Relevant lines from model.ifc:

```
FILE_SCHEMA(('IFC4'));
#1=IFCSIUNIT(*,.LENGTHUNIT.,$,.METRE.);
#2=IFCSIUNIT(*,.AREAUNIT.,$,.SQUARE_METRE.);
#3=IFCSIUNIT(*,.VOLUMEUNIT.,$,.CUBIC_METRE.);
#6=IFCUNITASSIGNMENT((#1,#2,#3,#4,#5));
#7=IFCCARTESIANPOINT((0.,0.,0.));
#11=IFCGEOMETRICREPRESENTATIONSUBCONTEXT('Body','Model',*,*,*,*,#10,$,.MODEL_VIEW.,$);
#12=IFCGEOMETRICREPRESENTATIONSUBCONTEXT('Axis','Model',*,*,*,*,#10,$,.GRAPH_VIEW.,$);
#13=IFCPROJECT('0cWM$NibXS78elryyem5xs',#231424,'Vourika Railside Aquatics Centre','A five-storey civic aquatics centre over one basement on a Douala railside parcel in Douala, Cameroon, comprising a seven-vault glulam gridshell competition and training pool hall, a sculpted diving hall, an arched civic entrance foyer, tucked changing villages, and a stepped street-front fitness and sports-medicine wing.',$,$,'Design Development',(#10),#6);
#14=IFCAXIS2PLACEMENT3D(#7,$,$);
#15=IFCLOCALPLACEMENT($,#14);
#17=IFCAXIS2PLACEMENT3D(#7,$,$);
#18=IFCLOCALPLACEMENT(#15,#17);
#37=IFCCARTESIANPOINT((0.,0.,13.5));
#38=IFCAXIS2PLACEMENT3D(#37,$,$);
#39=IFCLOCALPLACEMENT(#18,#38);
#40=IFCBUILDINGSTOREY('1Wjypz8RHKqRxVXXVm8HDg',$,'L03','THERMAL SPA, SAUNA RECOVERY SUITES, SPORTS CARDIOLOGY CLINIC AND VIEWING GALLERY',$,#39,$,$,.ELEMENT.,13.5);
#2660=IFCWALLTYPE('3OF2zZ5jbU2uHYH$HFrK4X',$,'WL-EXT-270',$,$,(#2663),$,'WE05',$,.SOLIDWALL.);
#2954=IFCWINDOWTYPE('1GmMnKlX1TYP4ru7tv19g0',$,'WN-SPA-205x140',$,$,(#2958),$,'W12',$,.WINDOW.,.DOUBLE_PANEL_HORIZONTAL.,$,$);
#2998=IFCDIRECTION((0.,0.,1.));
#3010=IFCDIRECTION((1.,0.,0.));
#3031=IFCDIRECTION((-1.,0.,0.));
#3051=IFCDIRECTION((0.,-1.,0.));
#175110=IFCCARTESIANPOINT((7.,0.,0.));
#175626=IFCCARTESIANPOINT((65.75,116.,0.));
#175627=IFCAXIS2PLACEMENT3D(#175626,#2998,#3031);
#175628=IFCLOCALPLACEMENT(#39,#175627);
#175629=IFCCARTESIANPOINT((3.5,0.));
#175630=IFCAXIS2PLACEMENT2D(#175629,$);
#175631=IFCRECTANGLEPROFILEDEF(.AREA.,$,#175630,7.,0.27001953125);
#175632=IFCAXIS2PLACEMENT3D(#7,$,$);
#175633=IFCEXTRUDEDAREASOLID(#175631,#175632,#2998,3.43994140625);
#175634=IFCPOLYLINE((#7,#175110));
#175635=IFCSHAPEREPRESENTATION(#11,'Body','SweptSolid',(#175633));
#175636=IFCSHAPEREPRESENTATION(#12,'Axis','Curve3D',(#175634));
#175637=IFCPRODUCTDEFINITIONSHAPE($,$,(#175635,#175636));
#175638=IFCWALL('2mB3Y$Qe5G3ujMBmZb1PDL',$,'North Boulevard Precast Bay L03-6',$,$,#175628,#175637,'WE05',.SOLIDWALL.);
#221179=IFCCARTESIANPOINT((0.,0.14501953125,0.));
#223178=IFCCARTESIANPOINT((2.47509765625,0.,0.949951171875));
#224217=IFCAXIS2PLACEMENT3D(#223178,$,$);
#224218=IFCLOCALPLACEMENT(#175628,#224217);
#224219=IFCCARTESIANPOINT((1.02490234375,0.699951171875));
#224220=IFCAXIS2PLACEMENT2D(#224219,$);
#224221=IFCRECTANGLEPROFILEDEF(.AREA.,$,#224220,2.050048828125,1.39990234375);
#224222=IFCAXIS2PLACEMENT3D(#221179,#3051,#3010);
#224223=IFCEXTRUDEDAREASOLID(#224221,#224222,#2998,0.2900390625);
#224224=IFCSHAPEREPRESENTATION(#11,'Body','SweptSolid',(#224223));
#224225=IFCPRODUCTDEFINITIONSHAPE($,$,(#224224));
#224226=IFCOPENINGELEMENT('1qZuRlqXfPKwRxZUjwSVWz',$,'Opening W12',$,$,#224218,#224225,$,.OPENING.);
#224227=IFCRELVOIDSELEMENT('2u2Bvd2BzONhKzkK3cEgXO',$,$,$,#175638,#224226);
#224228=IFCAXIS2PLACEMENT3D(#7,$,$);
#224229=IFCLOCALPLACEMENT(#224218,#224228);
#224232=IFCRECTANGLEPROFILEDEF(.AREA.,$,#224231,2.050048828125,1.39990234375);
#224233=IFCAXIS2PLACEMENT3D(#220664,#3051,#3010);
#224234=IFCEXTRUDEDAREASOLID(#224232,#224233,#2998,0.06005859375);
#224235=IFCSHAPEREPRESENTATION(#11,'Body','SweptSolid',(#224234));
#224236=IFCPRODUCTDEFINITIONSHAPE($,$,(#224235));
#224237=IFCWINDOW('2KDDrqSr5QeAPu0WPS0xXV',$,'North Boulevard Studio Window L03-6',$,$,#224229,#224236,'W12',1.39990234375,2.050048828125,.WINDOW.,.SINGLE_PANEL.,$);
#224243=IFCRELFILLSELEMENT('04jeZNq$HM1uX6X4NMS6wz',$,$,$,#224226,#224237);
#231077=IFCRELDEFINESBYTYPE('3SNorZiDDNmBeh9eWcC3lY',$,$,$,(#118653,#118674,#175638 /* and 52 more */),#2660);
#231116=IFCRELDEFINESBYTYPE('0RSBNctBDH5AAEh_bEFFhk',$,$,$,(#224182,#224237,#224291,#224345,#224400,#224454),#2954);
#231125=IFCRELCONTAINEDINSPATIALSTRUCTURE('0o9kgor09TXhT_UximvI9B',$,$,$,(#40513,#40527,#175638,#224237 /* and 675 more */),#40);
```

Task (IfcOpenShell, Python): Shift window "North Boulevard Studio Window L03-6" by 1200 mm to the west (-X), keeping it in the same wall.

```python
import ifcopenshell
import ifcopenshell.api.geometry
import ifcopenshell.util.placement

model = ifcopenshell.open("model.ifc")

window = model.by_id(224237)
opening = window.FillsVoids[0].RelatingOpeningElement
wall = opening.VoidsElements[0].RelatingBuildingElement

wall_matrix = ifcopenshell.util.placement.get_local_placement(wall.ObjectPlacement)
shift = wall_matrix[:3, 0] * 1.2
before = ifcopenshell.util.placement.get_local_placement(window.ObjectPlacement)[:3, 3].copy()

# The window is placed relative to its opening, so it follows when the opening moves.
matrix = ifcopenshell.util.placement.get_local_placement(opening.ObjectPlacement)
matrix[:3, 3] += shift
ifcopenshell.api.geometry.edit_object_placement(
    model, product=opening, matrix=matrix, is_si=False, should_transform_children=True
)

after = ifcopenshell.util.placement.get_local_placement(window.ObjectPlacement)[:3, 3]
print("window moved by", (after - before).round(3) + 0.0)

model.write("model-out.ifc")
```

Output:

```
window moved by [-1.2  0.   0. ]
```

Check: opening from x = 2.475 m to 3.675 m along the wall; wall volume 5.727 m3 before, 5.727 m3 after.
